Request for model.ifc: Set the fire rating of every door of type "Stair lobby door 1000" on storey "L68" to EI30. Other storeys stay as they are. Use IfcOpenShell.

First a look at what the model holds.

```python
import ifcopenshell
import ifcopenshell.util.element

model = ifcopenshell.open("model.ifc")
print(model.schema)
storey = next(s for s in model.by_type("IfcBuildingStorey") if s.Name == "L68")
doors = [e for e in ifcopenshell.util.element.get_decomposition(storey) if e.is_a("IfcDoor")]
seen = {}
for e in doors:
    element_type = ifcopenshell.util.element.get_type(e)
    key = (element_type.Name if element_type != e and element_type else None, ifcopenshell.util.element.get_pset(e, "Pset_DoorCommon", "FireRating"))
    seen[key] = seen.get(key, 0) + 1
for (name, value), count in sorted(seen.items(), key=str):
    print(count, "x", name, "|", value)
```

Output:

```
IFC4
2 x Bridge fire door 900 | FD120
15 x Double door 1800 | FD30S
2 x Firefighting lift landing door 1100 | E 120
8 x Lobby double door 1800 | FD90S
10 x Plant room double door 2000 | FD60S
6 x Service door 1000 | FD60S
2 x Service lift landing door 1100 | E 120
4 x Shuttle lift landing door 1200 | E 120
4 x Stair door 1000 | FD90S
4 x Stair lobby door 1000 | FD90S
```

```python
import ifcopenshell
import ifcopenshell.api.pset
import ifcopenshell.util.element

model = ifcopenshell.open("model.ifc")

storey = next(s for s in model.by_type("IfcBuildingStorey") if s.Name == "L68")
doors = [e for e in ifcopenshell.util.element.get_decomposition(storey) if e.is_a("IfcDoor")]

count = 0
for e in doors:
    element_type = ifcopenshell.util.element.get_type(e)
    if element_type in (None, e) or element_type.Name != "Stair lobby door 1000":
        continue
    # add_pset returns the element's existing set when there is one.
    pset = ifcopenshell.api.pset.add_pset(model, product=e, name="Pset_DoorCommon")
    ifcopenshell.api.pset.edit_pset(model, pset=pset, properties={"FireRating": "EI30"})
    count += 1

print(count, "doors updated")

model.write("model-out.ifc")
```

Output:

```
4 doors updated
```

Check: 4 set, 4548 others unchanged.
